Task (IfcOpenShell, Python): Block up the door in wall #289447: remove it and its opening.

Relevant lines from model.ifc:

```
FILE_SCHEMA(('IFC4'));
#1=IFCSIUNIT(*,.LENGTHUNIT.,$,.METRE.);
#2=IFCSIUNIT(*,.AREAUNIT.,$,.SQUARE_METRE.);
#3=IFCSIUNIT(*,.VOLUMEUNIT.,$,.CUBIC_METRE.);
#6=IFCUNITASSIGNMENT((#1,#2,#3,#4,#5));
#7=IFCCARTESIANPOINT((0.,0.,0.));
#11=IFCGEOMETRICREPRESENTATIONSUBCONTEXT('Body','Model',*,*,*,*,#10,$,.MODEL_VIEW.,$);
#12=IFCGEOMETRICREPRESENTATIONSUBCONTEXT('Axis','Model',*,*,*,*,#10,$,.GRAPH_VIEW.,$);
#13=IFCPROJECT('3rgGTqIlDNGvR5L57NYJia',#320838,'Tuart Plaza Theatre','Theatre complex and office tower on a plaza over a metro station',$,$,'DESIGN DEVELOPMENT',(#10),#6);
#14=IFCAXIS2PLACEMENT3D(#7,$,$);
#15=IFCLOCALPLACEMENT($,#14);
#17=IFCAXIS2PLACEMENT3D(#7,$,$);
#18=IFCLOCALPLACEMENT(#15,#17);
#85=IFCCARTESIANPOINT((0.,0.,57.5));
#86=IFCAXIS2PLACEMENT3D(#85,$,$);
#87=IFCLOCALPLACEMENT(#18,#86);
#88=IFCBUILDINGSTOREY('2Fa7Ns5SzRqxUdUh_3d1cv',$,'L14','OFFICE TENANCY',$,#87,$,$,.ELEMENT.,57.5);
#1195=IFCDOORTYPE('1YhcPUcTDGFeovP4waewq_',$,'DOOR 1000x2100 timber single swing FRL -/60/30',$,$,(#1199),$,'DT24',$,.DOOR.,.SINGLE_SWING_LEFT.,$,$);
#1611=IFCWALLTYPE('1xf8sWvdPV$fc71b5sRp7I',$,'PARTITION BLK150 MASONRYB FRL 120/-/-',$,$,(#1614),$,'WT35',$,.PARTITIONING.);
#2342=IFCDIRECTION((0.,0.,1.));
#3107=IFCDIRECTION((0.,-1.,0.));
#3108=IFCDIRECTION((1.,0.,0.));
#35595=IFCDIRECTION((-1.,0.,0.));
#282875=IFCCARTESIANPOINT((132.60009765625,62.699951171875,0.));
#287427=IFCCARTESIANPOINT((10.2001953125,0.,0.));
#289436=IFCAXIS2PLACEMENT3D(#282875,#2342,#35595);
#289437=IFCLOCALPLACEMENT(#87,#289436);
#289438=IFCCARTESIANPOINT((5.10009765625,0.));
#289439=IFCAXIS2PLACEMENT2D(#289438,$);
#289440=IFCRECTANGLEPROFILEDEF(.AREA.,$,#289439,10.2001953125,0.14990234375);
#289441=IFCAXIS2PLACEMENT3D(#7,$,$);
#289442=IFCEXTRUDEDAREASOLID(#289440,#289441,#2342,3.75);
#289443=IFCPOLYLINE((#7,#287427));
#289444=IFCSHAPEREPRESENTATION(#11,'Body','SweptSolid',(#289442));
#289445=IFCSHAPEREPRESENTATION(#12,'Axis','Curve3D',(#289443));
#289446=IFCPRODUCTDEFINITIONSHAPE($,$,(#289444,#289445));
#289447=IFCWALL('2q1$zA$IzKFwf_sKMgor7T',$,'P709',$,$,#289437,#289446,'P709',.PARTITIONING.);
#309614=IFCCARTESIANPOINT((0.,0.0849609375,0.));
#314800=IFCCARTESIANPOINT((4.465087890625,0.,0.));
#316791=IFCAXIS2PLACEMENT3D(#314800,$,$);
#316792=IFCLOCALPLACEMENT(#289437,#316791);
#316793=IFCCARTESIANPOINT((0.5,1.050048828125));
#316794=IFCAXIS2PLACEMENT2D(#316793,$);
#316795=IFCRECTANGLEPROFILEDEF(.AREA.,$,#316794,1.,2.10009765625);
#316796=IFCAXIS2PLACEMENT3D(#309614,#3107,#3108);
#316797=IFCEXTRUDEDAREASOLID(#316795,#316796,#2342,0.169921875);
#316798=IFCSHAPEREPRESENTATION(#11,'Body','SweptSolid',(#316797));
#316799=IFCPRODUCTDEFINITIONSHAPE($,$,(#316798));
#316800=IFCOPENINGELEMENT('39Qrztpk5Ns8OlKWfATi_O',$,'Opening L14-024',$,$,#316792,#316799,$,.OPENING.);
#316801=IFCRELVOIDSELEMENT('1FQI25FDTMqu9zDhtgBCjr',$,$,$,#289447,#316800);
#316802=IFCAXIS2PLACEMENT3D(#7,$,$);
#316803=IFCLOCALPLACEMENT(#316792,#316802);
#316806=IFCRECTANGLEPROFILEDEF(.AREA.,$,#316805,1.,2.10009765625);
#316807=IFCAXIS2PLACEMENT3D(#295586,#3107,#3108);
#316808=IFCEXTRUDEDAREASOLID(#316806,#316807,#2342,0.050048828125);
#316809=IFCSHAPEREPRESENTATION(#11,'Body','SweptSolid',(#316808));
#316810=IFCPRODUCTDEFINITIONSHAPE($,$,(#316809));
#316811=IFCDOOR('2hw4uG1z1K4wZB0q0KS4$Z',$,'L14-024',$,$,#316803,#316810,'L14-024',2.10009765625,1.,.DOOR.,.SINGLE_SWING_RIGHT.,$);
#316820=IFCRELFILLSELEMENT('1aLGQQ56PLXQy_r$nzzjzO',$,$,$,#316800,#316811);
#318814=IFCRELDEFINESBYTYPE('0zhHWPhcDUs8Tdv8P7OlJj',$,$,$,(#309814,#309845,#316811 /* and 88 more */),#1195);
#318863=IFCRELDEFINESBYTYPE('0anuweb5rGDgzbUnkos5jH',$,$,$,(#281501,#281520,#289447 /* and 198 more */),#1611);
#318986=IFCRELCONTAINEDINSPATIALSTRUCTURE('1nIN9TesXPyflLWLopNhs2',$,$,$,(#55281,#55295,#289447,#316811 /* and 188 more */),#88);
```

```python
import ifcopenshell
import ifcopenshell.api.feature
import ifcopenshell.api.root
import ifcopenshell.geom
import ifcopenshell.util.shape

model = ifcopenshell.open("model.ifc")
settings = ifcopenshell.geom.settings()


def volume(element):
    """Net volume in cubic metres, openings subtracted."""
    shape = ifcopenshell.geom.create_shape(settings, element)
    return ifcopenshell.util.shape.get_volume(shape.geometry)


door = model.by_guid("2hw4uG1z1K4wZB0q0KS4$Z")
opening = door.FillsVoids[0].RelatingOpeningElement
wall = opening.VoidsElements[0].RelatingBuildingElement
before = volume(wall)

ifcopenshell.api.root.remove_product(model, product=door)
ifcopenshell.api.feature.remove_feature(model, feature=opening)

after = volume(wall)

print(f"wall volume {before:.3f} -> {after:.3f} m3")

model.write("model_edited.ifc")
```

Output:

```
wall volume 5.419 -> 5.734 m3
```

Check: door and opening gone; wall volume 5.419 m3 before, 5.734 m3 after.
